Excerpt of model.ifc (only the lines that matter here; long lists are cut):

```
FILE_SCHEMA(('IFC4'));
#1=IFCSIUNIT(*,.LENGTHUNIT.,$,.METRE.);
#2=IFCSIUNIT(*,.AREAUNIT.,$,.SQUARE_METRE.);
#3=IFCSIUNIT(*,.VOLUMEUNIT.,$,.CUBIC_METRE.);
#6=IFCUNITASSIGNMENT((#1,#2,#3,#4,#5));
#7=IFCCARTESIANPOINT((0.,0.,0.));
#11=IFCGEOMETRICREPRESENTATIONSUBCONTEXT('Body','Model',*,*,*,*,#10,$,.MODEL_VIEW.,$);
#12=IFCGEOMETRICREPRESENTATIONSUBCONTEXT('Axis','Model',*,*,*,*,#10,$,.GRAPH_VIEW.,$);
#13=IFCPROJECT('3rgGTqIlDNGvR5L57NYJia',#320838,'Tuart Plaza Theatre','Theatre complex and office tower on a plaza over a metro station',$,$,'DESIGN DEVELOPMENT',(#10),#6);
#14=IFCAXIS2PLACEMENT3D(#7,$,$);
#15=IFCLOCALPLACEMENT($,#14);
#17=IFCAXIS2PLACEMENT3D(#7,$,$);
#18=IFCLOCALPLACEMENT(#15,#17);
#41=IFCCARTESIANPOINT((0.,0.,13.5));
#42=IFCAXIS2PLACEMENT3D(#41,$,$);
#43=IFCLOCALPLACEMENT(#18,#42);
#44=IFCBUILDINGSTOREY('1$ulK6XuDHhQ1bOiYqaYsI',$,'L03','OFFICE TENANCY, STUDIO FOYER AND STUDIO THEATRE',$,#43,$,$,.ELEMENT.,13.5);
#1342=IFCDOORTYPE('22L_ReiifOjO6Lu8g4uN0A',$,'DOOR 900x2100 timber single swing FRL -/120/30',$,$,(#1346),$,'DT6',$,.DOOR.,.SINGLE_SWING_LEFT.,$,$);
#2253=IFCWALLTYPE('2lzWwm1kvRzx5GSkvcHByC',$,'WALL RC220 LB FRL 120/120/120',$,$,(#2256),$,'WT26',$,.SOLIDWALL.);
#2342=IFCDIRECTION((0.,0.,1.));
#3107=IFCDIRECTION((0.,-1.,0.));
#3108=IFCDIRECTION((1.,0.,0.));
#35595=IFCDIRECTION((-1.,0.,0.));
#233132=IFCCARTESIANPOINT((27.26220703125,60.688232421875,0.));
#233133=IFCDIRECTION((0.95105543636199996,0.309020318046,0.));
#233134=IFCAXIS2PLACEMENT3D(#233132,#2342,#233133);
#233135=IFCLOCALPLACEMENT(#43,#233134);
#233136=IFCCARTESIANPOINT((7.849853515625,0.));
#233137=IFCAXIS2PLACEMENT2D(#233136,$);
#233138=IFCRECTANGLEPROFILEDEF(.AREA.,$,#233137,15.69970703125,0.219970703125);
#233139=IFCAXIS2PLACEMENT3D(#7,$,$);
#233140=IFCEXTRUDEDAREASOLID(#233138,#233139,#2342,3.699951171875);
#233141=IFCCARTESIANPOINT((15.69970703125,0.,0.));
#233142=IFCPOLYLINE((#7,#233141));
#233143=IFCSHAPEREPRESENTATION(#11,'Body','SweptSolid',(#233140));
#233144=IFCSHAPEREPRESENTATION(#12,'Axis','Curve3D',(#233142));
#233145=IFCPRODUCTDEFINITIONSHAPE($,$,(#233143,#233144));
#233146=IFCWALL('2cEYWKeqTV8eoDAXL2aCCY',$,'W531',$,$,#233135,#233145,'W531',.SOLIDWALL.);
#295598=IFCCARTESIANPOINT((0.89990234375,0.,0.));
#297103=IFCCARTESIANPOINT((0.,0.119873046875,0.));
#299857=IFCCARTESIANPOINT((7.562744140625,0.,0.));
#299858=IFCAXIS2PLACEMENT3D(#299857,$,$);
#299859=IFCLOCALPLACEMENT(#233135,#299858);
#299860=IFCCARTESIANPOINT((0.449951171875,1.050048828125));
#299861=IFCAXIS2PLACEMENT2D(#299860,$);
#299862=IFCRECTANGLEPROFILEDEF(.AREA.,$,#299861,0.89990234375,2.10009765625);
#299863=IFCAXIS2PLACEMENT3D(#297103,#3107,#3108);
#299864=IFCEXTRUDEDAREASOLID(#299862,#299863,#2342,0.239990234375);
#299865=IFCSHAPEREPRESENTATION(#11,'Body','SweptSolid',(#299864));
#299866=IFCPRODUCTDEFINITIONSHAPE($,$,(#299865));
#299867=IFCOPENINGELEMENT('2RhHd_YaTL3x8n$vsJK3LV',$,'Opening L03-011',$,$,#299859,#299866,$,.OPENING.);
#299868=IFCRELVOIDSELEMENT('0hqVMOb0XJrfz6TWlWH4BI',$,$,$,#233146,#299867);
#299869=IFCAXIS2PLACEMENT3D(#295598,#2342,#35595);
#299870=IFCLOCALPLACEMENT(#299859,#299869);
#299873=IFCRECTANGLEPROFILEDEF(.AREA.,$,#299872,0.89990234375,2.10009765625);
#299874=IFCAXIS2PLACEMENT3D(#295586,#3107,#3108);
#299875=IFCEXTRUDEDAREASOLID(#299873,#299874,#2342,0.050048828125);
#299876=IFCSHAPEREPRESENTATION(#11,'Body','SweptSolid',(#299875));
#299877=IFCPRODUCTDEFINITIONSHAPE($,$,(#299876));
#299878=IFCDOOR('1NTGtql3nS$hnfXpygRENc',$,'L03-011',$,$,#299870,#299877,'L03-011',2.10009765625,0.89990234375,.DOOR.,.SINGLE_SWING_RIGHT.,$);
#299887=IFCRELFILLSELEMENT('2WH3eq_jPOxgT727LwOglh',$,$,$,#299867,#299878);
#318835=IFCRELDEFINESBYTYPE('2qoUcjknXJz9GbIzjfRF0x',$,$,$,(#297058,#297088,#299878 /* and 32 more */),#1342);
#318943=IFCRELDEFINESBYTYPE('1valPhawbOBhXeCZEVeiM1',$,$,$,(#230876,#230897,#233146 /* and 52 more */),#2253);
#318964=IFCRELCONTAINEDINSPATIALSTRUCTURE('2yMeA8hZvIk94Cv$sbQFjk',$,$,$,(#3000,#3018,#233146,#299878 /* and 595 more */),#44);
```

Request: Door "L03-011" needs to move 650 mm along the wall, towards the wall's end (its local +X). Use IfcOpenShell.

```python
import ifcopenshell
import ifcopenshell.api.geometry
import ifcopenshell.util.placement
import ifcopenshell.util.unit

model = ifcopenshell.open("model.ifc")
unit_scale = ifcopenshell.util.unit.calculate_unit_scale(model)

door = model.by_guid("1NTGtql3nS$hnfXpygRENc")
opening = door.FillsVoids[0].RelatingOpeningElement
wall = opening.VoidsElements[0].RelatingBuildingElement

wall_matrix = ifcopenshell.util.placement.get_local_placement(wall.ObjectPlacement)
shift = wall_matrix[:3, 0] * 0.65 / unit_scale
before = ifcopenshell.util.placement.get_local_placement(door.ObjectPlacement)[:3, 3].copy()

# The door is placed relative to its opening, so it follows when the opening moves.
matrix = ifcopenshell.util.placement.get_local_placement(opening.ObjectPlacement)
matrix[:3, 3] += shift
ifcopenshell.api.geometry.edit_object_placement(
    model, product=opening, matrix=matrix, is_si=False, should_transform_children=True
)

after = ifcopenshell.util.placement.get_local_placement(door.ObjectPlacement)[:3, 3]
print("door moved by", (after - before).round(3) + 0.0)

model.write("model_updated.ifc")
```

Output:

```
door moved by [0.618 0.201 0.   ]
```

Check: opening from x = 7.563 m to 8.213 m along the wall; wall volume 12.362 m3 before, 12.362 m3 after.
